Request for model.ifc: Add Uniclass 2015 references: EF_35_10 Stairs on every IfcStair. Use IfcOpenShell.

First a look at what the model holds.

```python
import ifcopenshell

model = ifcopenshell.open("model.ifc")
print(model.schema)
print("classifications:", [c.Name for c in model.by_type("IfcClassification")])
for ifc_class in ("IfcDoor", "IfcRoof", "IfcStair", "IfcWall", "IfcWindow"):
    print(ifc_class, len(model.by_type(ifc_class)))
```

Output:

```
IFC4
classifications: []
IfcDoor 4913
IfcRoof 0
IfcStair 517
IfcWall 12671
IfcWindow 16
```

```python
import ifcopenshell
import ifcopenshell.api.classification

model = ifcopenshell.open("model.ifc")

system = ifcopenshell.api.classification.add_classification(model, classification="Uniclass 2015")

codes = {
    "IfcStair": ("EF_35_10", "Stairs"),
}
for ifc_class, (code, name) in codes.items():
    products = model.by_type(ifc_class)
    ifcopenshell.api.classification.add_reference(
        model, products=products, classification=system, identification=code, name=name
    )
    print(code, len(products))

model.write("model_rev.ifc")
```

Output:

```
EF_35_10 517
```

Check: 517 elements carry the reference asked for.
